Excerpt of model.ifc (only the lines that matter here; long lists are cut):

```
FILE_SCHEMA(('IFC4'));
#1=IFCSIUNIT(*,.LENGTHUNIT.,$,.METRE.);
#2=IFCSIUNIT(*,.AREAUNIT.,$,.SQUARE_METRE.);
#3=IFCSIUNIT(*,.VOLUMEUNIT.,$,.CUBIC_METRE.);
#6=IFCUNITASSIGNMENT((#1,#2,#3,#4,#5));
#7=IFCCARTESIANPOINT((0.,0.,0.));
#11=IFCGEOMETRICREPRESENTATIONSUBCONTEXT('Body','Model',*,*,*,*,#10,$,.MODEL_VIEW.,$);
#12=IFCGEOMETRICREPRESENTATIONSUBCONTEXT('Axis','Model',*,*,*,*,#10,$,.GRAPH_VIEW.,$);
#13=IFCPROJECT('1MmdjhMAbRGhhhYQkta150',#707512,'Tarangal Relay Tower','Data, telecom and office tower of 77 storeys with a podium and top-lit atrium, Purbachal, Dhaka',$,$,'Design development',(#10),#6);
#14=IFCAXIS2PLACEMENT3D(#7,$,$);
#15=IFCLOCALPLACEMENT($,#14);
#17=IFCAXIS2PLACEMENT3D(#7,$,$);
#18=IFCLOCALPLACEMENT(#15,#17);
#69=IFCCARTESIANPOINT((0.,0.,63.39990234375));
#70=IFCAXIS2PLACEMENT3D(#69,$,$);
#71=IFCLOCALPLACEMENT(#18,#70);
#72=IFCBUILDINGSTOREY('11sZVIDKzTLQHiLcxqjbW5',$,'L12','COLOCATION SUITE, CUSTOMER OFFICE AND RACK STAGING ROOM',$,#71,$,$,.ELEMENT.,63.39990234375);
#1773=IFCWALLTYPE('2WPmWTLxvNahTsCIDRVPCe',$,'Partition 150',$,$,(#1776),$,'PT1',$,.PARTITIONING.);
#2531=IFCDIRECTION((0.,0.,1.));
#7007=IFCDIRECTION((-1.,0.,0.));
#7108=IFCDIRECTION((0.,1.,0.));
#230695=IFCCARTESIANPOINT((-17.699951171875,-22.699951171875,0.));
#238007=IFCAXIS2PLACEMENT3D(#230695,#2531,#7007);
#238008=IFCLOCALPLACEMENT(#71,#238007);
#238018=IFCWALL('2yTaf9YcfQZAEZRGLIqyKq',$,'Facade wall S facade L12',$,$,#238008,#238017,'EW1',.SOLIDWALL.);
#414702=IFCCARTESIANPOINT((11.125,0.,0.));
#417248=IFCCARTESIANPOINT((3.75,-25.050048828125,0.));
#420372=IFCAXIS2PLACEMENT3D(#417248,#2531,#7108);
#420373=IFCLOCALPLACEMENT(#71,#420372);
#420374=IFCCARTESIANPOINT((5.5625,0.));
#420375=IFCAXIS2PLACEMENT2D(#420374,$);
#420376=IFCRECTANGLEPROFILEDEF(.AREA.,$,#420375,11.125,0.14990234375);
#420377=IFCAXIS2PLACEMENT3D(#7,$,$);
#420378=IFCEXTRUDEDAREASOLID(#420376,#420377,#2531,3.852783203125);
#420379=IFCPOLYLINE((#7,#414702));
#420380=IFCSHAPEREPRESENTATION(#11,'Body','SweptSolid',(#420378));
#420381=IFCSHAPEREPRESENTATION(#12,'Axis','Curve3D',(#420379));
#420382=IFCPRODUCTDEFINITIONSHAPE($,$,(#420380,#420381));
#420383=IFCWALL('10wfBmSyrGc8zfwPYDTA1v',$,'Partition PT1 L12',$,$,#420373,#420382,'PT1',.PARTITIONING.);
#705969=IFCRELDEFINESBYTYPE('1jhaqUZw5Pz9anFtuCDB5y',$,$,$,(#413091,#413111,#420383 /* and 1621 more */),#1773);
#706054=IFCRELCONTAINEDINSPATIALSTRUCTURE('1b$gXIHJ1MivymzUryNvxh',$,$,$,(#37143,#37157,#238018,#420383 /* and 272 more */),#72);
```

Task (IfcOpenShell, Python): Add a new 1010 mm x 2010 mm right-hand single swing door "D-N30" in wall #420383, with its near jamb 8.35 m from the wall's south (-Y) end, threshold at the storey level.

```python
import numpy as np
import ifcopenshell
import ifcopenshell.api.feature
import ifcopenshell.api.geometry
import ifcopenshell.api.root
import ifcopenshell.api.spatial
import ifcopenshell.geom
import ifcopenshell.util.element
import ifcopenshell.util.placement
import ifcopenshell.util.representation
import ifcopenshell.util.shape
import ifcopenshell.util.unit

model = ifcopenshell.open("model.ifc")
unit_scale = ifcopenshell.util.unit.calculate_unit_scale(model)
settings = ifcopenshell.geom.settings()


def volume(element):
    """Net volume in cubic metres, openings subtracted."""
    shape = ifcopenshell.geom.create_shape(settings, element)
    return ifcopenshell.util.shape.get_volume(shape.geometry)


wall = model.by_id(420383)
storey = ifcopenshell.util.element.get_container(wall, ifc_class="IfcBuildingStorey")
context = ifcopenshell.util.representation.get_context(model, "Model", "Body", "MODEL_VIEW")
before = volume(wall)

width, height, from_end, sill = 1.01, 2.01, 8.35, 0.0  # metres

# The wall runs along its own X axis, and the end named is its -X end.
wall_shape = ifcopenshell.geom.create_shape(settings, wall)
x, y, z = ifcopenshell.util.shape.get_vertices(wall_shape.geometry).T
start = x.min() + from_end
face, thickness = float(y.min()), float(y.max() - y.min())
wall_matrix = ifcopenshell.util.placement.get_local_placement(wall.ObjectPlacement)
level = ifcopenshell.util.placement.get_local_placement(storey.ObjectPlacement)[2, 3]


def in_wall(x, y):
    """Placement at x, y metres in the wall's axes, at sill height."""
    matrix = wall_matrix.copy()
    matrix[:, 3] = wall_matrix @ np.array([x / unit_scale, y / unit_scale, 0.0, 1.0])
    matrix[2, 3] = level + sill / unit_scale
    return matrix


# Opening: a box that overshoots both wall faces by 50 mm.
opening = ifcopenshell.api.root.create_entity(model, ifc_class="IfcOpeningElement", predefined_type="OPENING")
box = ifcopenshell.api.geometry.add_wall_representation(
    model, context=context, length=width, height=height, thickness=thickness + 0.1
)
ifcopenshell.api.geometry.assign_representation(model, product=opening, representation=box)
ifcopenshell.api.geometry.edit_object_placement(model, product=opening, matrix=in_wall(start, face - 0.05), is_si=False)
ifcopenshell.api.feature.add_feature(model, feature=opening, element=wall)

door = ifcopenshell.api.root.create_entity(model, ifc_class="IfcDoor", name="D-N30", predefined_type="DOOR")
door.OverallWidth, door.OverallHeight = width / unit_scale, height / unit_scale
door.OperationType = "SINGLE_SWING_RIGHT"
body = ifcopenshell.api.geometry.add_door_representation(
    model,
    context=context,
    overall_width=door.OverallWidth,
    overall_height=door.OverallHeight,
    operation_type="SINGLE_SWING_RIGHT",
    lining_properties={"LiningDepth": thickness / unit_scale, "ThresholdDepth": thickness / unit_scale},
)
ifcopenshell.api.geometry.assign_representation(model, product=door, representation=body)
ifcopenshell.api.spatial.assign_container(model, products=[door], relating_structure=storey)
ifcopenshell.api.feature.add_filling(model, opening=opening, element=door)

# The lining spans the wall, so the door starts at the wall face.
ifcopenshell.api.geometry.edit_object_placement(model, product=door, matrix=in_wall(start, face), is_si=False)

after = volume(wall)

print(f"wall volume {before:.3f} -> {after:.3f} m3")

model.write("model_updated.ifc")
```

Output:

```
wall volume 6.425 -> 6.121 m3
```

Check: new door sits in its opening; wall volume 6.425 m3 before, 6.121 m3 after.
